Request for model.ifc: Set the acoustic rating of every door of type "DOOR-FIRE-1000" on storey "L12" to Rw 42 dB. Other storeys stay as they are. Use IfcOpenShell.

First a look at what the model holds.

```python
import ifcopenshell
import ifcopenshell.util.element

model = ifcopenshell.open("model.ifc")
print(model.schema)
storey = next(s for s in model.by_type("IfcBuildingStorey") if s.Name == "L12")
doors = [e for e in ifcopenshell.util.element.get_decomposition(storey) if e.is_a("IfcDoor")]
seen = {}
for e in doors:
    element_type = ifcopenshell.util.element.get_type(e)
    key = (element_type.Name if element_type != e and element_type else None, ifcopenshell.util.element.get_pset(e, "Pset_DoorCommon", "AcousticRating"))
    seen[key] = seen.get(key, 0) + 1
for (name, value), count in sorted(seen.items(), key=str):
    print(count, "x", name, "|", value)
```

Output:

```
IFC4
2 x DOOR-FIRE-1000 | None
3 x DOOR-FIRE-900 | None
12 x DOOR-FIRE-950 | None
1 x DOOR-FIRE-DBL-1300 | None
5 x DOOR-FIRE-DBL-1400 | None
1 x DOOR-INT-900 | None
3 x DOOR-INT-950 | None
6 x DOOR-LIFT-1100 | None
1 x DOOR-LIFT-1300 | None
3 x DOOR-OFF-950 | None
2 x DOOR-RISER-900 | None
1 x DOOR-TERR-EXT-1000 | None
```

```python
import ifcopenshell
import ifcopenshell.api.pset
import ifcopenshell.util.element

model = ifcopenshell.open("model.ifc")

storey = next(s for s in model.by_type("IfcBuildingStorey") if s.Name == "L12")
doors = [e for e in ifcopenshell.util.element.get_decomposition(storey) if e.is_a("IfcDoor")]

count = 0
for e in doors:
    element_type = ifcopenshell.util.element.get_type(e)
    if element_type in (None, e) or element_type.Name != "DOOR-FIRE-1000":
        continue
    # add_pset returns the element's existing set when there is one.
    pset = ifcopenshell.api.pset.add_pset(model, product=e, name="Pset_DoorCommon")
    ifcopenshell.api.pset.edit_pset(model, pset=pset, properties={"AcousticRating": "Rw 42 dB"})
    count += 1

print(count, "doors updated")

model.write("model_rev.ifc")
```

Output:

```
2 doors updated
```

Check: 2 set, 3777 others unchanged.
